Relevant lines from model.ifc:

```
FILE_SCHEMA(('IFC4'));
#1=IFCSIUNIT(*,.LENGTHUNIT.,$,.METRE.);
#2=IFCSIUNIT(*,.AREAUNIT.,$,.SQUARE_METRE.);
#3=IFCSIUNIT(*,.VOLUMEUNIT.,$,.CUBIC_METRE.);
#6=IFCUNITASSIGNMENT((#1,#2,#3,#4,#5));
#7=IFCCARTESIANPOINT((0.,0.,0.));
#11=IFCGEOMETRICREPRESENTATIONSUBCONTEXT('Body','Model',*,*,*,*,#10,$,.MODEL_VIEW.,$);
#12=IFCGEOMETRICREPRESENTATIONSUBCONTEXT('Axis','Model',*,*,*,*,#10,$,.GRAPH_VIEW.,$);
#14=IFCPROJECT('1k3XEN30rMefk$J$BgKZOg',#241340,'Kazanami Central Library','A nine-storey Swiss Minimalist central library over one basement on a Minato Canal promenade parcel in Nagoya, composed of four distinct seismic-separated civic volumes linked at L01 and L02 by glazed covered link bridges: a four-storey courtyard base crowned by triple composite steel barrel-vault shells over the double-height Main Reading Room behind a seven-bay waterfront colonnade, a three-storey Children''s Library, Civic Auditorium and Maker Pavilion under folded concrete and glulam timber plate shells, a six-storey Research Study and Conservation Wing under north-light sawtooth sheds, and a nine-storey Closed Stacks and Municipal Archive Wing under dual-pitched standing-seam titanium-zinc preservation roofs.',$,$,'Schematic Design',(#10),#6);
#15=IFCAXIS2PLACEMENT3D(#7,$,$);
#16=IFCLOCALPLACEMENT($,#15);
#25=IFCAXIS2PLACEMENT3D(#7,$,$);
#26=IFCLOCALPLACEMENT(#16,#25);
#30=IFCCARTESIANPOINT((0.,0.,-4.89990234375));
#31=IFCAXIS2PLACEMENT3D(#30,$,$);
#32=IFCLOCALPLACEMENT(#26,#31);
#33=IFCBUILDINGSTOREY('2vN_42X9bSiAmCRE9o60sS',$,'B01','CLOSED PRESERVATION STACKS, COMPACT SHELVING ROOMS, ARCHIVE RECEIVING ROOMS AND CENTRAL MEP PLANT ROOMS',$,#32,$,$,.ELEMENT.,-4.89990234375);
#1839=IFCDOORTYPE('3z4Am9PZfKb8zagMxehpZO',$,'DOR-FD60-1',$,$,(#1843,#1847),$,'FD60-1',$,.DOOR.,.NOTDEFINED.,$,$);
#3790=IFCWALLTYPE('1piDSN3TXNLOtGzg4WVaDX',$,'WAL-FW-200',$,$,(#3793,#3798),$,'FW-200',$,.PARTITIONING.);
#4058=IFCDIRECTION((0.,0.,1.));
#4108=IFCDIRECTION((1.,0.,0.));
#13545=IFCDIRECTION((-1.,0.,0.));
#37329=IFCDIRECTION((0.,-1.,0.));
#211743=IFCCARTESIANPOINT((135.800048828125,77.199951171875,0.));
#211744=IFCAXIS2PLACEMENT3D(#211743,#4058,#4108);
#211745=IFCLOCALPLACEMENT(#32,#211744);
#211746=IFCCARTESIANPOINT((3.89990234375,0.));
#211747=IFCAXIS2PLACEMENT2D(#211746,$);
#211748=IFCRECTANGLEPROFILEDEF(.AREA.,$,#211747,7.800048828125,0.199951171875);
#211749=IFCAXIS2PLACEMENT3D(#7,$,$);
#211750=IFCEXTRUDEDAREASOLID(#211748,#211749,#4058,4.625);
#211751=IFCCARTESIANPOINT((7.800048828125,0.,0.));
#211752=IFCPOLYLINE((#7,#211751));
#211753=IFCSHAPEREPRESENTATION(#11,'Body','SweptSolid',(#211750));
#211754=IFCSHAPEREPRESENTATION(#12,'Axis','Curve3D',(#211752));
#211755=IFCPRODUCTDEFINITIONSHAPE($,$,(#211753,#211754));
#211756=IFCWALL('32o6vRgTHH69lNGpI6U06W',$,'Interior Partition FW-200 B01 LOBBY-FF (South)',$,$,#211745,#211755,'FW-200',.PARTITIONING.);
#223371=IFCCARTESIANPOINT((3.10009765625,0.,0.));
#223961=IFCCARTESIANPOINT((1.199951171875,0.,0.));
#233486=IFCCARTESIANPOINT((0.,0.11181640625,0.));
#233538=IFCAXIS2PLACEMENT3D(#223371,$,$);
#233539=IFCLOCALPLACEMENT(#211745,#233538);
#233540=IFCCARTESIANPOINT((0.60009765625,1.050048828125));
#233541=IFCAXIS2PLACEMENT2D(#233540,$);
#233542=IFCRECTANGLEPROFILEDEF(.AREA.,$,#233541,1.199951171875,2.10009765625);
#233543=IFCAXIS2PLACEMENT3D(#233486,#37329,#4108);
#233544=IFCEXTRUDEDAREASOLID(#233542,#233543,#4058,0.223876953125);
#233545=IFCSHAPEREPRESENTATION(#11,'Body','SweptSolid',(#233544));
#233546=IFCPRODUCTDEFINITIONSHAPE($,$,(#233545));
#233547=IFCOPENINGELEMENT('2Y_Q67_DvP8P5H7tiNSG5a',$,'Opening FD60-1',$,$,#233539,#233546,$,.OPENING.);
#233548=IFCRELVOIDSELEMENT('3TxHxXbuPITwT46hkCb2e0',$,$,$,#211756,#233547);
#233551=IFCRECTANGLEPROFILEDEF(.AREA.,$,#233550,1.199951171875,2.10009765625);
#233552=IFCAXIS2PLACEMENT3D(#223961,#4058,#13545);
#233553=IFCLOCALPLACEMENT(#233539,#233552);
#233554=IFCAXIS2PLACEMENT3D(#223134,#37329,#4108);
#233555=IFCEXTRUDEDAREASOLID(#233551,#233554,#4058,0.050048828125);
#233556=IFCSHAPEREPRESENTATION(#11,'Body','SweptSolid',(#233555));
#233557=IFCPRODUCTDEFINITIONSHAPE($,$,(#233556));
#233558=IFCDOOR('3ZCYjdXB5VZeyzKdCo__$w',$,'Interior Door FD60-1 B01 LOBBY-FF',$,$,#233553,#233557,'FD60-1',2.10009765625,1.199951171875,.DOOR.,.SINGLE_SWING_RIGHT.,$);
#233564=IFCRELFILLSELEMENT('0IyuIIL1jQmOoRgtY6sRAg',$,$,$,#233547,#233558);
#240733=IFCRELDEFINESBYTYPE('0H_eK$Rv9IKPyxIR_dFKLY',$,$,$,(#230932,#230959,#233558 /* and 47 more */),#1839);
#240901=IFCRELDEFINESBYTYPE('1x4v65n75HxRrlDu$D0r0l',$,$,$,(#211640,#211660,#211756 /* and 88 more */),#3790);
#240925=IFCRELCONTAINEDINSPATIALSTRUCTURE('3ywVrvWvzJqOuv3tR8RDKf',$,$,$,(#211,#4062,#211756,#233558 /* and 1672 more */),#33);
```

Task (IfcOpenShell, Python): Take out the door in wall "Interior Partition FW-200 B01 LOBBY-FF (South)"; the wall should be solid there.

```python
import ifcopenshell
import ifcopenshell.api.feature
import ifcopenshell.api.root
import ifcopenshell.geom
import ifcopenshell.util.shape

model = ifcopenshell.open("model.ifc")
settings = ifcopenshell.geom.settings()


def volume(element):
    """Net volume in cubic metres, openings subtracted."""
    shape = ifcopenshell.geom.create_shape(settings, element)
    return ifcopenshell.util.shape.get_volume(shape.geometry)


door = model.by_guid("3ZCYjdXB5VZeyzKdCo__$w")
opening = door.FillsVoids[0].RelatingOpeningElement
wall = opening.VoidsElements[0].RelatingBuildingElement
before = volume(wall)

ifcopenshell.api.root.remove_product(model, product=door)
ifcopenshell.api.feature.remove_feature(model, feature=opening)

after = volume(wall)

print(f"wall volume {before:.3f} -> {after:.3f} m3")

model.write("model_v2.ifc")
```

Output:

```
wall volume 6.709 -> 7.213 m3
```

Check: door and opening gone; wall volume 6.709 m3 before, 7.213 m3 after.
